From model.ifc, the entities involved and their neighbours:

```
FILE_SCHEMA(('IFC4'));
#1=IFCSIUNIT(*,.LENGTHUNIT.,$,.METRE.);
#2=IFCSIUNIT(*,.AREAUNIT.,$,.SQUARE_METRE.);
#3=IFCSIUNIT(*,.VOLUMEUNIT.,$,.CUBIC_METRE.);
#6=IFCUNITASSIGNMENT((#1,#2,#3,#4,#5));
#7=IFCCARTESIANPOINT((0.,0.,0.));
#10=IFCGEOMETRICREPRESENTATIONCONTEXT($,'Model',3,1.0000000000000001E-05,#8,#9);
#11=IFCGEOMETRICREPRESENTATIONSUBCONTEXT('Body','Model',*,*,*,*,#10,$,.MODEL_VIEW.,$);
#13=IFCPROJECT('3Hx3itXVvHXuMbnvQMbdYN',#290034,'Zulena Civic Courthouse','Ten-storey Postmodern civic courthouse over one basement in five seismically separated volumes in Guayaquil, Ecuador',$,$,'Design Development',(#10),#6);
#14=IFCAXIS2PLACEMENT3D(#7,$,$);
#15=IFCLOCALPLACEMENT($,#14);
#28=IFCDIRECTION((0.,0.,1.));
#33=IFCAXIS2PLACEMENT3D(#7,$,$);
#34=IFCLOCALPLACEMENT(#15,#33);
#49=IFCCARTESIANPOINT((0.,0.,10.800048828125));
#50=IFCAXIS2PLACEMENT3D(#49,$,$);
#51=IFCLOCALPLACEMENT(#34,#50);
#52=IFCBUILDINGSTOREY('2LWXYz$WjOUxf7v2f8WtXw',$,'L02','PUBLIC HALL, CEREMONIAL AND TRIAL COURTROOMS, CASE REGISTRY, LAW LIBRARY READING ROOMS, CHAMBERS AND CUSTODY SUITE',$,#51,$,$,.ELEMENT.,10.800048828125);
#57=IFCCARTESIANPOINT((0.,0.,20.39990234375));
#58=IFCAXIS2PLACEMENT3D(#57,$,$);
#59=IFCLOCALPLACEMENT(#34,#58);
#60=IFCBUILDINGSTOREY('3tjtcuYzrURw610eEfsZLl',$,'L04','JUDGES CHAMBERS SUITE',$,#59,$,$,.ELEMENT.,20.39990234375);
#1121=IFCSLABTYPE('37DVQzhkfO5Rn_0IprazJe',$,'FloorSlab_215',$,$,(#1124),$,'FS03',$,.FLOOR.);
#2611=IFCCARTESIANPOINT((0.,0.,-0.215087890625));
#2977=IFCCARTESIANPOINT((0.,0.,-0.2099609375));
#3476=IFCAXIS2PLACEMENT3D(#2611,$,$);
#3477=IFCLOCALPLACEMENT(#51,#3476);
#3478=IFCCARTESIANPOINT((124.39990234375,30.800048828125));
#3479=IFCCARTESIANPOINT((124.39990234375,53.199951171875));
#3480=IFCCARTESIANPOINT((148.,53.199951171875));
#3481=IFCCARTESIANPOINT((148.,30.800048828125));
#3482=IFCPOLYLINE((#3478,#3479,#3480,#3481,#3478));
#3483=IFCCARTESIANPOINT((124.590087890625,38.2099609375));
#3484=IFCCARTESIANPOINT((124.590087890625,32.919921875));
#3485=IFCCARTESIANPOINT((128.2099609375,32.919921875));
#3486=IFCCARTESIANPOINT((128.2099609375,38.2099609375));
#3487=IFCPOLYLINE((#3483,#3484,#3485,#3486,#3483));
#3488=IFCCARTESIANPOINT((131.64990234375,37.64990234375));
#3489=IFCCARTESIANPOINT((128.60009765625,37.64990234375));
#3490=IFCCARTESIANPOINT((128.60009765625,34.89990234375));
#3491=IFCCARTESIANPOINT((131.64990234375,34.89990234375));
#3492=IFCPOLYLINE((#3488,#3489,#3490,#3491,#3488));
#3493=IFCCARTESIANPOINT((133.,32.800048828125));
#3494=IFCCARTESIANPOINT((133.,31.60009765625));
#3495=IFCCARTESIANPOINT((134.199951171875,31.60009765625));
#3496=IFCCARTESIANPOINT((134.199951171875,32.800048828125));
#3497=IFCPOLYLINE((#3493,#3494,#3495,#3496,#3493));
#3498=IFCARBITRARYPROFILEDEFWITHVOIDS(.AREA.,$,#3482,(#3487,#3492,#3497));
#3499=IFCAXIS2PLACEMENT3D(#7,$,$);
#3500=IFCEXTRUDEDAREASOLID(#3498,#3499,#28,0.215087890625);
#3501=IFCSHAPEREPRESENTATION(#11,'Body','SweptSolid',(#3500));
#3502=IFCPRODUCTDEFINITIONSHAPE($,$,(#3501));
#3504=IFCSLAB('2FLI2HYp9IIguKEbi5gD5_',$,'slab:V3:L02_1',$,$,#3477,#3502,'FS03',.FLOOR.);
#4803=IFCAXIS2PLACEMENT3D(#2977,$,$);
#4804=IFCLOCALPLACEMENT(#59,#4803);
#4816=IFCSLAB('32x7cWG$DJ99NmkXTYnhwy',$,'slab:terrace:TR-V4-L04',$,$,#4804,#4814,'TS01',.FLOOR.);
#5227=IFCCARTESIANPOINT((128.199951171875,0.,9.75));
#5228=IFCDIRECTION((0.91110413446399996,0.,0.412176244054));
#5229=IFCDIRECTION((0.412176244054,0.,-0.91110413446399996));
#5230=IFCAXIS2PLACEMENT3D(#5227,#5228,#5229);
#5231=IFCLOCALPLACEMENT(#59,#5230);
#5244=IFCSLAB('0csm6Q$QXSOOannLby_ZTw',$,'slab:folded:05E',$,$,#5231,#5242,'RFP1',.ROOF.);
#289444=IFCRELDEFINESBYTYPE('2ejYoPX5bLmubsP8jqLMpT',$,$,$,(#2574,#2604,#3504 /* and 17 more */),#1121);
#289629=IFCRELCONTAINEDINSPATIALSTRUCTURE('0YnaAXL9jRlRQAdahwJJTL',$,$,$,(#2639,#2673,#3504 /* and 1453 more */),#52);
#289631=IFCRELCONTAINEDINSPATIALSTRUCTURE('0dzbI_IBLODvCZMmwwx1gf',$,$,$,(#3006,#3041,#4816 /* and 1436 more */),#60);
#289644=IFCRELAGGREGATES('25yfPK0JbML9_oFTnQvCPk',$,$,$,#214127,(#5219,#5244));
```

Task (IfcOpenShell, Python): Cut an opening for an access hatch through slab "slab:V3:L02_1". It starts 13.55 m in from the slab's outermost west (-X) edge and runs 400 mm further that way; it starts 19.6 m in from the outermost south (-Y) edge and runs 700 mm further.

```python
import numpy as np
import ifcopenshell
import ifcopenshell.api.feature
import ifcopenshell.api.geometry
import ifcopenshell.api.root
import ifcopenshell.geom
import ifcopenshell.util.placement
import ifcopenshell.util.representation
import ifcopenshell.util.shape
import ifcopenshell.util.unit

model = ifcopenshell.open("model.ifc")
unit_scale = ifcopenshell.util.unit.calculate_unit_scale(model)
settings = ifcopenshell.geom.settings()


def volume(element):
    """Net volume in cubic metres, openings subtracted."""
    shape = ifcopenshell.geom.create_shape(settings, element)
    return ifcopenshell.util.shape.get_volume(shape.geometry)


slab = model.by_guid("2FLI2HYp9IIguKEbi5gD5_")
before = volume(slab)

# Extent in the slab's own axes, in metres. The edges named are its -X and -Y sides.
slab_shape = ifcopenshell.geom.create_shape(settings, slab)
vertices = ifcopenshell.util.shape.get_vertices(slab_shape.geometry)
x_min, y_min, bottom = vertices.min(axis=0)
top = vertices[:, 2].max()

opening = ifcopenshell.api.root.create_entity(model, ifc_class="IfcOpeningElement", name="Access hatch opening", predefined_type="OPENING")
context = ifcopenshell.util.representation.get_context(model, "Model", "Body", "MODEL_VIEW")
width, depth = 0.4, 0.7
outline = [(0.0, 0.0), (width, 0.0), (width, depth), (0.0, depth), (0.0, 0.0)]
# Overshoot both faces by 50 mm so the cut is clean.
shape = ifcopenshell.api.geometry.add_slab_representation(
    model, context=context, depth=top - bottom + 0.1, polyline=outline
)
ifcopenshell.api.geometry.assign_representation(model, product=opening, representation=shape)

matrix = ifcopenshell.util.placement.get_local_placement(slab.ObjectPlacement)
matrix[:, 3] = matrix @ np.append(np.array([x_min + 13.55, y_min + 19.6, bottom - 0.05]) / unit_scale, 1.0)
ifcopenshell.api.geometry.edit_object_placement(model, product=opening, matrix=matrix, is_si=False)
ifcopenshell.api.feature.add_feature(model, feature=opening, element=slab)

after = volume(slab)

print(f"slab volume {before:.3f} -> {after:.3f} m3")

model.write("model_rev.ifc")
```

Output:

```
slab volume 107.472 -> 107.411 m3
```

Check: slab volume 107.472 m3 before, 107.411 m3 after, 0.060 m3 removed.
